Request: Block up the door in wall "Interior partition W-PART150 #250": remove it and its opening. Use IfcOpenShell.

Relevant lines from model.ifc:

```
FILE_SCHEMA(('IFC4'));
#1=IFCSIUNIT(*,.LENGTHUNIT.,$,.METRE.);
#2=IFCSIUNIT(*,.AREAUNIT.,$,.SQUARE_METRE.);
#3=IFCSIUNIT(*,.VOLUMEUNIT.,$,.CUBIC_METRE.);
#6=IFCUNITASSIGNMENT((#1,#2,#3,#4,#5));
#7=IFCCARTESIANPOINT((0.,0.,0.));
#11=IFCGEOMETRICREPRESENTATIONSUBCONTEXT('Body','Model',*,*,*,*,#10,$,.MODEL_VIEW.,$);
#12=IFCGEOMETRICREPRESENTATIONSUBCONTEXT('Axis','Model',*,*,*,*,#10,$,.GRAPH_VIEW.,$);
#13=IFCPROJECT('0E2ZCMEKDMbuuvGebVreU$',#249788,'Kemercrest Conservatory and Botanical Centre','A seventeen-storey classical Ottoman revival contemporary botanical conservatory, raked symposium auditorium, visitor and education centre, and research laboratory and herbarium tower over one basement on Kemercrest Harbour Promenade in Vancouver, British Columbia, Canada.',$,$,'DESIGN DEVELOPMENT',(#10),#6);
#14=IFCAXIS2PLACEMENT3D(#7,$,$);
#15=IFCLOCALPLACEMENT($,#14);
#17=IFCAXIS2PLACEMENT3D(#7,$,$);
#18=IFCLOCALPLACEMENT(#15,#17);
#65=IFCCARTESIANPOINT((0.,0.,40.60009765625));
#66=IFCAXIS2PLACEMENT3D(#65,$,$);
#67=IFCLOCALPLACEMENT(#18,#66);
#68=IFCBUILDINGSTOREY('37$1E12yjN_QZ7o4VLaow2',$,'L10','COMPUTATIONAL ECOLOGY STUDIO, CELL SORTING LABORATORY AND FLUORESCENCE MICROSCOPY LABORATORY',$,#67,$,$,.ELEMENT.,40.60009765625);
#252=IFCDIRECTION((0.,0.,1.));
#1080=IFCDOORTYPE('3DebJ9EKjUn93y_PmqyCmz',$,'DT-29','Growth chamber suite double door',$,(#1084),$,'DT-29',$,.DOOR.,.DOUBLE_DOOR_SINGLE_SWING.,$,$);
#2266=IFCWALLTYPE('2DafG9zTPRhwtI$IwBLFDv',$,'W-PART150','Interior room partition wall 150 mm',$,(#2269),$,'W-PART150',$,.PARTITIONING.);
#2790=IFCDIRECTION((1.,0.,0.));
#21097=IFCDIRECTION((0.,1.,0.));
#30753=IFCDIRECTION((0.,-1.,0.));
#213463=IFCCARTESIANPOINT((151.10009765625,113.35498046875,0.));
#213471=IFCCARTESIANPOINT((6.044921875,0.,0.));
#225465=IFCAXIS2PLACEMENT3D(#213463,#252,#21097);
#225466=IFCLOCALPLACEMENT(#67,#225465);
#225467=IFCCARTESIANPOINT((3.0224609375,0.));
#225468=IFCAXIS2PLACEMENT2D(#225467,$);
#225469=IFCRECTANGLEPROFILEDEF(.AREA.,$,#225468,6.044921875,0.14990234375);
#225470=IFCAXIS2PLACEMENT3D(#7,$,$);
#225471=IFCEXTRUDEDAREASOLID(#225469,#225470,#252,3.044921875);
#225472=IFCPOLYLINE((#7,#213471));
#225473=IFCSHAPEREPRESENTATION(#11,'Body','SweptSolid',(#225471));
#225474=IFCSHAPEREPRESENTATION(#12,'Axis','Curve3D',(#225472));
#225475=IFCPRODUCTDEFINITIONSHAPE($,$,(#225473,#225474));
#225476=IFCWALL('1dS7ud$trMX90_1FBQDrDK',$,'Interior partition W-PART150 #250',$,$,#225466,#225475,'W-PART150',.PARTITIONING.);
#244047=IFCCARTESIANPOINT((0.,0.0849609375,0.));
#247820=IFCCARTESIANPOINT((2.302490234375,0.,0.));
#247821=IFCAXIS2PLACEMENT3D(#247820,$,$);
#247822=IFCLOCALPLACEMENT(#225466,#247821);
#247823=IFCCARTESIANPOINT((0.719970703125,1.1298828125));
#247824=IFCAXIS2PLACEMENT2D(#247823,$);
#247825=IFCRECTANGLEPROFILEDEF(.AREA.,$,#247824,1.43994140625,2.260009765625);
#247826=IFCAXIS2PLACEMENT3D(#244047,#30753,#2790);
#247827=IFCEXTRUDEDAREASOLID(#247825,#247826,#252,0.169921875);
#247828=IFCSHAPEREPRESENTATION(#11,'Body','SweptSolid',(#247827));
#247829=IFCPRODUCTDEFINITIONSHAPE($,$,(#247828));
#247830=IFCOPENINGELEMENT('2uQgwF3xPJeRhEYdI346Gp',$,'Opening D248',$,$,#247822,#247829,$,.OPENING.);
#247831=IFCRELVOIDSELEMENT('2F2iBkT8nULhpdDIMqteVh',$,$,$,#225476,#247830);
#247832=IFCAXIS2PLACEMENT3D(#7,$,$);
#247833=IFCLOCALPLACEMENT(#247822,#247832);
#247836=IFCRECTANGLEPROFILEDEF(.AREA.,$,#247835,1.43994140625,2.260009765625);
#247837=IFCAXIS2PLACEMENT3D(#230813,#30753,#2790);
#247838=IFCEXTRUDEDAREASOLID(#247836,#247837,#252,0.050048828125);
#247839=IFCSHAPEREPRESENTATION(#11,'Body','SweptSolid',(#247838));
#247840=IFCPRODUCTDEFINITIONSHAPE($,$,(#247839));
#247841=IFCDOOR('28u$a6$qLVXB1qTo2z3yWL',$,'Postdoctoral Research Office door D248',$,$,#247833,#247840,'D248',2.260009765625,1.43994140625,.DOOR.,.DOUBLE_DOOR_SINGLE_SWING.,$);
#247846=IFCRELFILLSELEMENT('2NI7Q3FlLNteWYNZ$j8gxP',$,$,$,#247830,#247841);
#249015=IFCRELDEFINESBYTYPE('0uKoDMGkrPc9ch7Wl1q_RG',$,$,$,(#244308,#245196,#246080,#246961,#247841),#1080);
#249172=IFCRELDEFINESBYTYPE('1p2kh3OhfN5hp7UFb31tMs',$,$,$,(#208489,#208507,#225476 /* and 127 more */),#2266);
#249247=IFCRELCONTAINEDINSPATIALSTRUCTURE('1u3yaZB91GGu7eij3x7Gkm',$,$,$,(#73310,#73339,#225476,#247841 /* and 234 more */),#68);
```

```python
import ifcopenshell
import ifcopenshell.api.feature
import ifcopenshell.api.root
import ifcopenshell.geom
import ifcopenshell.util.shape

model = ifcopenshell.open("model.ifc")
settings = ifcopenshell.geom.settings()


def volume(element):
    """Net volume in cubic metres, openings subtracted."""
    shape = ifcopenshell.geom.create_shape(settings, element)
    return ifcopenshell.util.shape.get_volume(shape.geometry)


door = model.by_guid("28u$a6$qLVXB1qTo2z3yWL")
opening = door.FillsVoids[0].RelatingOpeningElement
wall = opening.VoidsElements[0].RelatingBuildingElement
before = volume(wall)

ifcopenshell.api.root.remove_product(model, product=door)
ifcopenshell.api.feature.remove_feature(model, feature=opening)

after = volume(wall)

print(f"wall volume {before:.3f} -> {after:.3f} m3")

model.write("model_v2.ifc")
```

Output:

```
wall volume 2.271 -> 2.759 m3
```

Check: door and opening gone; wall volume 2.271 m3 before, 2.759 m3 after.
